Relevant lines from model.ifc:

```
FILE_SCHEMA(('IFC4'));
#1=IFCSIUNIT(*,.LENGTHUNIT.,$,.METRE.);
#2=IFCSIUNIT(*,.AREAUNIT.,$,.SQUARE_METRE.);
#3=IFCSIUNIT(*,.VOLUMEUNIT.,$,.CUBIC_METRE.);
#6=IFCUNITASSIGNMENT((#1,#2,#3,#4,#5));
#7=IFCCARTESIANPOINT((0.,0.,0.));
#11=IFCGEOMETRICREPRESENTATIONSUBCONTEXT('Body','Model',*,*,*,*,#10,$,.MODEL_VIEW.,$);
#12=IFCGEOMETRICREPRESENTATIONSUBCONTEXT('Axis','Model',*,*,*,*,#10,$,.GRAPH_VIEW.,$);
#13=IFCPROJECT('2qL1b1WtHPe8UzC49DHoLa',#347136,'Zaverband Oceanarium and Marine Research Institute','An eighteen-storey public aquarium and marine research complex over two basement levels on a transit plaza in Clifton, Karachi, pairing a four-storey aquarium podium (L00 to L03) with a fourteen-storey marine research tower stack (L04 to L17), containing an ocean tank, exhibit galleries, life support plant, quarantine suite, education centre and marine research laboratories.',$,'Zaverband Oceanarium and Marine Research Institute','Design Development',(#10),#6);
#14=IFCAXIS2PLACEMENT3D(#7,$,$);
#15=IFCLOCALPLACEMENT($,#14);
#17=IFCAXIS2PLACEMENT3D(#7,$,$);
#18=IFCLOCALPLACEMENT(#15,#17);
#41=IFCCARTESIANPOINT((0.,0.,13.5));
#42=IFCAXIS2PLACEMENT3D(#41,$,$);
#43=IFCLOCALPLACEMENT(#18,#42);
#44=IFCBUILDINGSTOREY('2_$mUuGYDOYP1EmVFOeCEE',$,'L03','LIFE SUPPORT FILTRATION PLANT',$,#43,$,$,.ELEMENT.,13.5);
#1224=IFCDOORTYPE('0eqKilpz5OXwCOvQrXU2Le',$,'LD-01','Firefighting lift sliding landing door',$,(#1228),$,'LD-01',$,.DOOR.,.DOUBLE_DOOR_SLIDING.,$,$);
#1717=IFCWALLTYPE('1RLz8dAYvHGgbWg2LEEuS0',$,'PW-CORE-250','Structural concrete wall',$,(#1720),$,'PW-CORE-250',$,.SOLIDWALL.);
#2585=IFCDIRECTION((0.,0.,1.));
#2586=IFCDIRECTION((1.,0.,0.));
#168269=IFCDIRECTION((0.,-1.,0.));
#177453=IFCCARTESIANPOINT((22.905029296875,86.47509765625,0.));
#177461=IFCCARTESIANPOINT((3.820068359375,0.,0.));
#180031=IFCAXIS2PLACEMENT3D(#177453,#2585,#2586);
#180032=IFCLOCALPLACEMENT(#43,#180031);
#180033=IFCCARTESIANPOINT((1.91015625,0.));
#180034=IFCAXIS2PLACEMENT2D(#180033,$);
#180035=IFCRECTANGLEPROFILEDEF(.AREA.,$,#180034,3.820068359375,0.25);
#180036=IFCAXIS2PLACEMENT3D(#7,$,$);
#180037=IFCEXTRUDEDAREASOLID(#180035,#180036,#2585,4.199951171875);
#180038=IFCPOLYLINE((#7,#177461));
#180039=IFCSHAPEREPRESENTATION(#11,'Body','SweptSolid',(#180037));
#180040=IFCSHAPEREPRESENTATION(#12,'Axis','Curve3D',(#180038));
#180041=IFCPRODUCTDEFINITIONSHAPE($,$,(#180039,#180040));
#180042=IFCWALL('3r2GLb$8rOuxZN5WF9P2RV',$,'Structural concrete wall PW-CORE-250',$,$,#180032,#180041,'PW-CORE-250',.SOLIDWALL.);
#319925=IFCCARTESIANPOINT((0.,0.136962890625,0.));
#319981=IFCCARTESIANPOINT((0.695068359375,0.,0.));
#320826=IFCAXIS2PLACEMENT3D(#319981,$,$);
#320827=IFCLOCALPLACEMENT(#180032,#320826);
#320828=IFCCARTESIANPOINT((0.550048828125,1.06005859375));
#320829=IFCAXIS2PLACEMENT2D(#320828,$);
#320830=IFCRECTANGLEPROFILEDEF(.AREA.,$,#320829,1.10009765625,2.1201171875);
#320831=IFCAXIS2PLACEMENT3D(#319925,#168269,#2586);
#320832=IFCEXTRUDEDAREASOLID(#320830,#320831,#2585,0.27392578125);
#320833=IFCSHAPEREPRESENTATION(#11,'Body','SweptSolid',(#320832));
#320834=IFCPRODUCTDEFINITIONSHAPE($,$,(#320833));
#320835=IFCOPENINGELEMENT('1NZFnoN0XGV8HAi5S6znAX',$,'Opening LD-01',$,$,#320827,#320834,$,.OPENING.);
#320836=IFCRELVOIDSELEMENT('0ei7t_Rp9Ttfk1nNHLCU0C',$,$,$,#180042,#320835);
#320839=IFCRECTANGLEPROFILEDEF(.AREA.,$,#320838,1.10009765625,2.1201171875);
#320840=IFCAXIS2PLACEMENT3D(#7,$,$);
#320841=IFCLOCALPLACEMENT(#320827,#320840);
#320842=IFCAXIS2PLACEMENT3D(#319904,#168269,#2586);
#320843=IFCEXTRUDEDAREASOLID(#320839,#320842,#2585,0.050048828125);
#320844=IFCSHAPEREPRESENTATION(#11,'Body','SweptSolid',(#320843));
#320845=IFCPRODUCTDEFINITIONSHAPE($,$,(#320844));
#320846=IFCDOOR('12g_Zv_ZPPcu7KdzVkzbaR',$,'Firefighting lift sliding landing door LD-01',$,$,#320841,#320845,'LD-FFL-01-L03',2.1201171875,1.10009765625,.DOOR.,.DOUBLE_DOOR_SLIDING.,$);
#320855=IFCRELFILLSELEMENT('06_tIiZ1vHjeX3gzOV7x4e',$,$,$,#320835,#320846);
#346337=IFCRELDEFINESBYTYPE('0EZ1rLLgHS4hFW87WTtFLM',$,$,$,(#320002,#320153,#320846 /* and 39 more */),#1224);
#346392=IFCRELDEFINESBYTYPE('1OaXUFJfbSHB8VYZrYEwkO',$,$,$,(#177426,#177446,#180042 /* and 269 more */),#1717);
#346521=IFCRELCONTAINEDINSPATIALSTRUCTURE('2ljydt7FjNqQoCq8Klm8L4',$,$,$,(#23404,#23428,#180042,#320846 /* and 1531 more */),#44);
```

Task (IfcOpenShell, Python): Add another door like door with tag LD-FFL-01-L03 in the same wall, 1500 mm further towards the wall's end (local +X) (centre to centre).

```python
import ifcopenshell
import ifcopenshell.api.feature
import ifcopenshell.api.geometry
import ifcopenshell.api.root
import ifcopenshell.geom
import ifcopenshell.util.element
import ifcopenshell.util.placement
import ifcopenshell.util.shape
import ifcopenshell.util.unit

model = ifcopenshell.open("model.ifc")
unit_scale = ifcopenshell.util.unit.calculate_unit_scale(model)
settings = ifcopenshell.geom.settings()


def volume(element):
    """Net volume in cubic metres, openings subtracted."""
    shape = ifcopenshell.geom.create_shape(settings, element)
    return ifcopenshell.util.shape.get_volume(shape.geometry)


door = model.by_guid("12g_Zv_ZPPcu7KdzVkzbaR")
opening = door.FillsVoids[0].RelatingOpeningElement
wall = opening.VoidsElements[0].RelatingBuildingElement
before = volume(wall)
shift = ifcopenshell.util.placement.get_local_placement(wall.ObjectPlacement)[:3, 0] * 1.5 / unit_scale

# copy_class copies the void relationship, type, container and properties, but no geometry.
new_opening = ifcopenshell.api.root.copy_class(model, product=opening)
new_opening.Representation = ifcopenshell.util.element.copy_deep(
    model, opening.Representation, exclude=["IfcGeometricRepresentationContext", "IfcRepresentationMap"]
)
new_door = ifcopenshell.api.root.copy_class(model, product=door)
new_door.Representation = ifcopenshell.util.element.copy_deep(
    model, door.Representation, exclude=["IfcGeometricRepresentationContext", "IfcRepresentationMap"]
)
new_door.Tag = None
ifcopenshell.api.feature.add_filling(model, opening=new_opening, element=new_door)

for old, new in ((opening, new_opening), (door, new_door)):
    matrix = ifcopenshell.util.placement.get_local_placement(old.ObjectPlacement)
    matrix[:3, 3] += shift
    ifcopenshell.api.geometry.edit_object_placement(model, product=new, matrix=matrix, is_si=False)

after = volume(wall)

print(f"wall volume {before:.3f} -> {after:.3f} m3")

model.write("model-out.ifc")
```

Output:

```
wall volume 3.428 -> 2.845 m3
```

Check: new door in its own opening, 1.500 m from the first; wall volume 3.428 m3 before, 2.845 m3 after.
